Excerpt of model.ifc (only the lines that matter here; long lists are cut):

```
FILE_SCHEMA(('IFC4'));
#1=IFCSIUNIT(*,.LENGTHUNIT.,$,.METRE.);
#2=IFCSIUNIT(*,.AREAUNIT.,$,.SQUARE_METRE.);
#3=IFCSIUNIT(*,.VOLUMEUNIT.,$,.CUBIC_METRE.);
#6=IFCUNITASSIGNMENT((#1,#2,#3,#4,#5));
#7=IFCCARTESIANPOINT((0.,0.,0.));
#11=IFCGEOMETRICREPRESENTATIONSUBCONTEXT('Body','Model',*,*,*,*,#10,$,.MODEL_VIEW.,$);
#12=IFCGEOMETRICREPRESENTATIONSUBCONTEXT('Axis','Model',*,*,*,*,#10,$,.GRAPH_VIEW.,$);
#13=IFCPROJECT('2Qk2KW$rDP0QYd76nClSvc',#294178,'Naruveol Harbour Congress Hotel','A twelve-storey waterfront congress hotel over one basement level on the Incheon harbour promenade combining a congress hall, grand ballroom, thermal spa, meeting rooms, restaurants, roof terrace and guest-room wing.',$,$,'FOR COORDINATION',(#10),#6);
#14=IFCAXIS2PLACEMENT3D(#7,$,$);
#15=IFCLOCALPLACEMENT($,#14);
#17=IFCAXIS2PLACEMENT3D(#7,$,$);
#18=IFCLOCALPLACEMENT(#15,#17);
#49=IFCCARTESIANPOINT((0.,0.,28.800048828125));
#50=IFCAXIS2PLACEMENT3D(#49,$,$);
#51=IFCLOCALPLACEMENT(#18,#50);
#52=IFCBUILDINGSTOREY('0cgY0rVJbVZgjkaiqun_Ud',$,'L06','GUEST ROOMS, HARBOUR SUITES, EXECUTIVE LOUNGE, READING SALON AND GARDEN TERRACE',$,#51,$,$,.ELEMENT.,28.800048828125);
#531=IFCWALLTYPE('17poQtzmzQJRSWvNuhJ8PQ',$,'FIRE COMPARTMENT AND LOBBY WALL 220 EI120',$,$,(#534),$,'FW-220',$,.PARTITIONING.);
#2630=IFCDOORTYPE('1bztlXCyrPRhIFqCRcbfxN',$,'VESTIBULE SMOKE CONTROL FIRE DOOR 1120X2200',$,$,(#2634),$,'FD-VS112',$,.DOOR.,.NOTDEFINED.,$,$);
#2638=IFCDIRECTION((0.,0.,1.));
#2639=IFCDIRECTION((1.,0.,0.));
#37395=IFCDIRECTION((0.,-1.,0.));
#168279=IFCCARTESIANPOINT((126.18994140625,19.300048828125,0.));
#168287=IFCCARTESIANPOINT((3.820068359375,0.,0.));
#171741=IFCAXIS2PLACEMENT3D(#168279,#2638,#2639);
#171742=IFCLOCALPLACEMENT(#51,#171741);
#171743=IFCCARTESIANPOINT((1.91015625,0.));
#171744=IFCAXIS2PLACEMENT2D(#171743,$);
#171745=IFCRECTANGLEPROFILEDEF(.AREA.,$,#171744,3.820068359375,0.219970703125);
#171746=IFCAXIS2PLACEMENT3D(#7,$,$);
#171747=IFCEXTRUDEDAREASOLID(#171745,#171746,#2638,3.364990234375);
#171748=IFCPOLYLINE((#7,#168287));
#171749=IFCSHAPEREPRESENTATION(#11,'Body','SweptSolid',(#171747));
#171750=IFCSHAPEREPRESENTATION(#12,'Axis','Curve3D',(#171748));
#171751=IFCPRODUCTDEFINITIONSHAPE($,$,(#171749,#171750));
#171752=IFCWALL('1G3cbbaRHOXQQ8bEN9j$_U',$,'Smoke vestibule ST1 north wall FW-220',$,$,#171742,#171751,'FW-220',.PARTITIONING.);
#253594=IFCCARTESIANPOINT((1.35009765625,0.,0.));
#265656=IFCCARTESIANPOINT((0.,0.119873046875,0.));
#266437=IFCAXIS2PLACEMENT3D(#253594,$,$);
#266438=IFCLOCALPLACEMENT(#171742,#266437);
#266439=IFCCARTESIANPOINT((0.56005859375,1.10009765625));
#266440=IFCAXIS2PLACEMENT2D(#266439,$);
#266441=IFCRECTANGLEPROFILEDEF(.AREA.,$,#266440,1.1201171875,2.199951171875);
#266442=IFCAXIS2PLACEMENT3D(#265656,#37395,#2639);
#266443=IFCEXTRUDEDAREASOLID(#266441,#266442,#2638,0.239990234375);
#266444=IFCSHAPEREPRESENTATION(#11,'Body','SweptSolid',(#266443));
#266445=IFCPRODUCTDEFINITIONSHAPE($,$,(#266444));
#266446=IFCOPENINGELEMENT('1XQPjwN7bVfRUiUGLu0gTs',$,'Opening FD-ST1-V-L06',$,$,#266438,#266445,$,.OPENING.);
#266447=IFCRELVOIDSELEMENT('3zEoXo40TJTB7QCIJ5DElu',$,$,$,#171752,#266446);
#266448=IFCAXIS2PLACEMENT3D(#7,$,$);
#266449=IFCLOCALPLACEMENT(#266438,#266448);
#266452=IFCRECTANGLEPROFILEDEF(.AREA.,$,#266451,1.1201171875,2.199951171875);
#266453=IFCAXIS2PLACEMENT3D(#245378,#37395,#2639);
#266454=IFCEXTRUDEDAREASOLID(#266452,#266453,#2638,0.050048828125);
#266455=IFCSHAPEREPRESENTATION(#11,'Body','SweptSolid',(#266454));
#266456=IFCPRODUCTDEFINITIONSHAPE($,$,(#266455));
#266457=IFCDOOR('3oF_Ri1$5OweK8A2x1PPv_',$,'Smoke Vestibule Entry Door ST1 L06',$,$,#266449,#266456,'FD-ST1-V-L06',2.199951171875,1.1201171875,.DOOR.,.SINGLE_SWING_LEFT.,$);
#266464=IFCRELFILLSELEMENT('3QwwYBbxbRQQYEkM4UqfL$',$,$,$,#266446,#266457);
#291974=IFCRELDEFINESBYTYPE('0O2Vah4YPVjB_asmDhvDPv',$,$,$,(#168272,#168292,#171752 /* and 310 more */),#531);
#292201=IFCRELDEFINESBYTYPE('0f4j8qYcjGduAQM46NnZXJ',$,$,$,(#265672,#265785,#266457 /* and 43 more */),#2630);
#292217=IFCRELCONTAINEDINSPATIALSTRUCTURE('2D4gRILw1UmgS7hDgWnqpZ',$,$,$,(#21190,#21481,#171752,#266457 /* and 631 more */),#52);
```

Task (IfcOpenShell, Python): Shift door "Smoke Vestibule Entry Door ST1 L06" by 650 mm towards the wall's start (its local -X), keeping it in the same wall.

```python
import ifcopenshell
import ifcopenshell.api.geometry
import ifcopenshell.util.placement

model = ifcopenshell.open("model.ifc")

door = model.by_guid("3oF_Ri1$5OweK8A2x1PPv_")
opening = door.FillsVoids[0].RelatingOpeningElement
wall = opening.VoidsElements[0].RelatingBuildingElement

wall_matrix = ifcopenshell.util.placement.get_local_placement(wall.ObjectPlacement)
shift = wall_matrix[:3, 0] * -0.65
before = ifcopenshell.util.placement.get_local_placement(door.ObjectPlacement)[:3, 3].copy()

# The door is placed relative to its opening, so it follows when the opening moves.
matrix = ifcopenshell.util.placement.get_local_placement(opening.ObjectPlacement)
matrix[:3, 3] += shift
ifcopenshell.api.geometry.edit_object_placement(
    model, product=opening, matrix=matrix, is_si=False, should_transform_children=True
)

after = ifcopenshell.util.placement.get_local_placement(door.ObjectPlacement)[:3, 3]
print("door moved by", (after - before).round(3) + 0.0)

model.write("model_v2.ifc")
```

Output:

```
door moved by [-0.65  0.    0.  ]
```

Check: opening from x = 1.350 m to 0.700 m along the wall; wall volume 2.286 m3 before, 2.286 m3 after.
